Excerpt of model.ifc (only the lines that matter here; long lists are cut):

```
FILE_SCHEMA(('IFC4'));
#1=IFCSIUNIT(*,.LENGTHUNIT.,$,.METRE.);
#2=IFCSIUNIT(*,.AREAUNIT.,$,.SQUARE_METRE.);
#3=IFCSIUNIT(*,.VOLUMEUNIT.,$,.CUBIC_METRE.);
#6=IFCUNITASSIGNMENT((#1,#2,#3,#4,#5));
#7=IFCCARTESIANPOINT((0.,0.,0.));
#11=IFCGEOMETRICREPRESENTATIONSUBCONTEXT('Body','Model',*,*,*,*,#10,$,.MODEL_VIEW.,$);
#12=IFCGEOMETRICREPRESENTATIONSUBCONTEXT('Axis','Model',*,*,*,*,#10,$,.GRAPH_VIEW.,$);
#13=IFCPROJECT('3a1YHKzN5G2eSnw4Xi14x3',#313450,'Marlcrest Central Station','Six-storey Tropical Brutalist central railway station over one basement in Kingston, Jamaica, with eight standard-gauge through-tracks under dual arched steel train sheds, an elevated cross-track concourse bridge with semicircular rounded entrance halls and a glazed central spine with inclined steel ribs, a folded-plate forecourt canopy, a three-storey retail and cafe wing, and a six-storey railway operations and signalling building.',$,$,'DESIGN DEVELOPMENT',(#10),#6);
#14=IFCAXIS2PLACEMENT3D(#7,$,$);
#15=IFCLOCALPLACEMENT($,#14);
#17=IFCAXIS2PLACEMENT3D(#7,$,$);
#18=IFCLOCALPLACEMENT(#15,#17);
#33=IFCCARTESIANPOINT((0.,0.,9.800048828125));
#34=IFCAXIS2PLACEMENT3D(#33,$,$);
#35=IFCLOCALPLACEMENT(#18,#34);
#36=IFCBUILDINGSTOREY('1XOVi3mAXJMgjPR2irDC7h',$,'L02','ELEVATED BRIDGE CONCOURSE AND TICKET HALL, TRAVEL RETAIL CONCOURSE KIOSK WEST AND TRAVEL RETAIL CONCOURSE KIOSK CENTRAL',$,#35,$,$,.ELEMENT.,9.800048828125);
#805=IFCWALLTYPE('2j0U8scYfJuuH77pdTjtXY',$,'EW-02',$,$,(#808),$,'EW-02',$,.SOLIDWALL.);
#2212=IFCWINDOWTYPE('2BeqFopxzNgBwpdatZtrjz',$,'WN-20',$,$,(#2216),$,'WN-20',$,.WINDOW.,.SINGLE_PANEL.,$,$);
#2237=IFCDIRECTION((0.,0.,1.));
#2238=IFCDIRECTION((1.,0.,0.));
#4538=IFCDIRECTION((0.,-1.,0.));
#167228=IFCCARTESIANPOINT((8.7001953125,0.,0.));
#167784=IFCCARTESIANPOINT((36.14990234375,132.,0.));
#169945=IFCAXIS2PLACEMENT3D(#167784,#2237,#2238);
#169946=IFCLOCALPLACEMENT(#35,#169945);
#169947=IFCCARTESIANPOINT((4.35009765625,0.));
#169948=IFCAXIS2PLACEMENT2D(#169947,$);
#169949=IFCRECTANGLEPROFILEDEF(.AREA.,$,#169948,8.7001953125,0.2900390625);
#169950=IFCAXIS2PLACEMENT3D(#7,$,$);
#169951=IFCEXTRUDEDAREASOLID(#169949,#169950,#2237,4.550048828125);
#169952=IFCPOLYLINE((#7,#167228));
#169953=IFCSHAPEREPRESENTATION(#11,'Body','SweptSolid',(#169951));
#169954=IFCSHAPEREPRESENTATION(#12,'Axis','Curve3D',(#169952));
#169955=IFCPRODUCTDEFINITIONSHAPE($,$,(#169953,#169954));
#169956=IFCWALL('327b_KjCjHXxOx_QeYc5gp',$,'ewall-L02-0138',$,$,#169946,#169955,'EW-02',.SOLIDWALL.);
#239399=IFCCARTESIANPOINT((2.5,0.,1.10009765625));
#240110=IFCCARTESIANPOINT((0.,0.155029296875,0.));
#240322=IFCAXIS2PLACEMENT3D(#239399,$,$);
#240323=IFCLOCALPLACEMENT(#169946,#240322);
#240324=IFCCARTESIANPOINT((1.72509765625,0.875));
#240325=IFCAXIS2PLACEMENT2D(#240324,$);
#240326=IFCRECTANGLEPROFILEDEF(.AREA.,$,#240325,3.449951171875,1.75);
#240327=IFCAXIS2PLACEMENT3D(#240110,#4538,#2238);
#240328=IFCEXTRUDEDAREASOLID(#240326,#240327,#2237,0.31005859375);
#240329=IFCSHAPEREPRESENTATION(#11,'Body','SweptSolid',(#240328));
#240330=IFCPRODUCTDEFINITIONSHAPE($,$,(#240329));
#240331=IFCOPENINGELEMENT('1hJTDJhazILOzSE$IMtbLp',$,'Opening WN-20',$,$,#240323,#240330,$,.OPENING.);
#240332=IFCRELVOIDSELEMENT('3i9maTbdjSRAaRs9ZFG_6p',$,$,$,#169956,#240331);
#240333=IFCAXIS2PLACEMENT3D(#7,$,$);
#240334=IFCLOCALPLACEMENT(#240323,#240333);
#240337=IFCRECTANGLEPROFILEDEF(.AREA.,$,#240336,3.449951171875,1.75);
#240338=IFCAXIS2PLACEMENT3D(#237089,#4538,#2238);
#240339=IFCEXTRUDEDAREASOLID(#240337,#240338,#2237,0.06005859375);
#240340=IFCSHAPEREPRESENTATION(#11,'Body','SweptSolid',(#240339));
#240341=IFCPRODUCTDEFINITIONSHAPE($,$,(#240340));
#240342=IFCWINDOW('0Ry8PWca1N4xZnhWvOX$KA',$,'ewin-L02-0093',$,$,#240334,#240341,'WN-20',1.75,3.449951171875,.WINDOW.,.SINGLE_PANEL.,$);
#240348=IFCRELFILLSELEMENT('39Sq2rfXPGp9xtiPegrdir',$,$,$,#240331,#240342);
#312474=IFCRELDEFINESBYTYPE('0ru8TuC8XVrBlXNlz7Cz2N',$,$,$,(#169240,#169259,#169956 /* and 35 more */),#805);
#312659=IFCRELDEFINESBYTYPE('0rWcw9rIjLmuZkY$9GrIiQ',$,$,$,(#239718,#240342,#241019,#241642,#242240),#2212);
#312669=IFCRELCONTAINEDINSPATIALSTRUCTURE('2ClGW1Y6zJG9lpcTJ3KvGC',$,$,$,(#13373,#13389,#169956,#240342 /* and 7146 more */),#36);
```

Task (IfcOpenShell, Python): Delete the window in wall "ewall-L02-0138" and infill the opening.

```python
import ifcopenshell
import ifcopenshell.api.feature
import ifcopenshell.api.root
import ifcopenshell.geom
import ifcopenshell.util.shape

model = ifcopenshell.open("model.ifc")
settings = ifcopenshell.geom.settings()


def volume(element):
    """Net volume in cubic metres, openings subtracted."""
    shape = ifcopenshell.geom.create_shape(settings, element)
    return ifcopenshell.util.shape.get_volume(shape.geometry)


window = model.by_guid("0Ry8PWca1N4xZnhWvOX$KA")
opening = window.FillsVoids[0].RelatingOpeningElement
wall = opening.VoidsElements[0].RelatingBuildingElement
before = volume(wall)

ifcopenshell.api.root.remove_product(model, product=window)
ifcopenshell.api.feature.remove_feature(model, feature=opening)

after = volume(wall)

print(f"wall volume {before:.3f} -> {after:.3f} m3")

model.write("model_edited.ifc")
```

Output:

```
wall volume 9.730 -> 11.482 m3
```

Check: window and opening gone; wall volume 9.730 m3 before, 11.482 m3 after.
